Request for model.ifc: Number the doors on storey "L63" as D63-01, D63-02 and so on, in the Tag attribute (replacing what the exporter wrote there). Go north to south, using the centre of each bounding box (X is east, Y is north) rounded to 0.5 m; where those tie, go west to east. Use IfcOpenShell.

First a look at what the model holds.

```python
import ifcopenshell
import ifcopenshell.util.element
import ifcopenshell.util.placement

model = ifcopenshell.open("model.ifc")
print(model.schema)
storey = next(s for s in model.by_type("IfcBuildingStorey") if s.Name == "L63")
doors = [e for e in ifcopenshell.util.element.get_decomposition(storey) if e.is_a("IfcDoor")]
for e in sorted(doors, key=lambda e: e.id()):
    origin = ifcopenshell.util.placement.get_local_placement(e.ObjectPlacement)[:3, 3]
    print(e.id(), e.Tag, e.Name, origin.round(2) + 0.0, sep=" | ")
```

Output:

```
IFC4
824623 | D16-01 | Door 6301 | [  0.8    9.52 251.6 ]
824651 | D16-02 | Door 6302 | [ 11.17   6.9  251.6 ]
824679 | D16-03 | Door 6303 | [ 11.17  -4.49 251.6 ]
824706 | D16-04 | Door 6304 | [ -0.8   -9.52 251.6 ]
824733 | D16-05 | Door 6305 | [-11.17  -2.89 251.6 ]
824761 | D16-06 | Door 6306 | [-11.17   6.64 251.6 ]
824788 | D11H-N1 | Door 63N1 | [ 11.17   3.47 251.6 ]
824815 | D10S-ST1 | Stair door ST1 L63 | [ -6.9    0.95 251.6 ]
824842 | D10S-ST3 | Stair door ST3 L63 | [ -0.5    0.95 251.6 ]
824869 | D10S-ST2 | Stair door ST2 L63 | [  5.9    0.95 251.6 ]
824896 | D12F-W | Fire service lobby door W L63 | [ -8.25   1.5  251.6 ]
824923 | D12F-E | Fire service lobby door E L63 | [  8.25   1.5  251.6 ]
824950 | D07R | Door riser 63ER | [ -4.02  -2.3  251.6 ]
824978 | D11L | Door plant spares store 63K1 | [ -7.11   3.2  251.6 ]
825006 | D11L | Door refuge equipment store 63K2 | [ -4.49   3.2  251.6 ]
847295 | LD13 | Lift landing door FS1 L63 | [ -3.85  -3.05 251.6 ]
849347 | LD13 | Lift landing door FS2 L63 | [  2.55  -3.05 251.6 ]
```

```python
import ifcopenshell
import ifcopenshell.geom
import ifcopenshell.util.element
import ifcopenshell.util.shape

model = ifcopenshell.open("model.ifc")
settings = ifcopenshell.geom.settings()
settings.set("use-world-coords", True)


def centre(element):
    shape = ifcopenshell.geom.create_shape(settings, element)
    return ifcopenshell.util.shape.get_bbox_centroid(shape.geometry)


storey = next(s for s in model.by_type("IfcBuildingStorey") if s.Name == "L63")
doors = [e for e in ifcopenshell.util.element.get_decomposition(storey) if e.is_a("IfcDoor")]

# Insertion points can sit at a corner or the storey origin, so sort by the geometry (in metres).
centres = {e: centre(e) for e in doors}
doors.sort(key=lambda e: (-round(centres[e][1] / 0.5), centres[e][0]))

for i, e in enumerate(doors, start=1):
    number = f"D63-{i:02d}"
    e.Tag = number
    print(e.id(), number)

model.write("model-out.ifc")
```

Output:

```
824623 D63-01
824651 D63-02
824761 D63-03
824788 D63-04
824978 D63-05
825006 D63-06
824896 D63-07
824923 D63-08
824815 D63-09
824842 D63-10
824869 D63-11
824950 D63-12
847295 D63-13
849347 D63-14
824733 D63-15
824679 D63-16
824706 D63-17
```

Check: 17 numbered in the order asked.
